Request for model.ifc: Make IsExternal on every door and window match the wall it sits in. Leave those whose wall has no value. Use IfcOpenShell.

First a look at what the model holds.

```python
import ifcopenshell
import ifcopenshell.util.element

model = ifcopenshell.open("model.ifc")
print(model.schema)
seen = {}
for e in model.by_type("IfcDoor") + model.by_type("IfcWindow"):
    if not e.FillsVoids:
        continue
    host = e.FillsVoids[0].RelatingOpeningElement.VoidsElements[0].RelatingBuildingElement
    own = ifcopenshell.util.element.get_pset(e, f"Pset_{e.is_a()[3:].removesuffix('StandardCase')}Common", "IsExternal")
    wall = ifcopenshell.util.element.get_pset(host, "Pset_WallCommon", "IsExternal")
    seen[e.is_a(), own, wall] = seen.get((e.is_a(), own, wall), 0) + 1
for (cls, own, wall), count in sorted(seen.items(), key=str):
    print(count, cls, "IsExternal:", own, "| host wall:", wall)
```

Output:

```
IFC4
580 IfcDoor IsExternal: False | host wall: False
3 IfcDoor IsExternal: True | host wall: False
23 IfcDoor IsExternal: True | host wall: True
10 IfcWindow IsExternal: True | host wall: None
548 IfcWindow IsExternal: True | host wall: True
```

```python
import ifcopenshell
import ifcopenshell.api.pset
import ifcopenshell.util.element

model = ifcopenshell.open("model.ifc")

count = 0
for ifc_class, pset_name in (("IfcDoor", "Pset_DoorCommon"), ("IfcWindow", "Pset_WindowCommon")):
    for e in model.by_type(ifc_class):
        if not e.FillsVoids:
            continue
        host = e.FillsVoids[0].RelatingOpeningElement.VoidsElements[0].RelatingBuildingElement
        external = ifcopenshell.util.element.get_pset(host, "Pset_WallCommon", "IsExternal")
        if external is None or ifcopenshell.util.element.get_pset(e, pset_name, "IsExternal") == external:
            continue
        pset = ifcopenshell.api.pset.add_pset(model, product=e, name=pset_name)
        ifcopenshell.api.pset.edit_pset(model, pset=pset, properties={"IsExternal": external})
        count += 1

print(count, "updated")

model.write("model_v2.ifc")
```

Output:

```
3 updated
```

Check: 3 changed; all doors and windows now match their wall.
